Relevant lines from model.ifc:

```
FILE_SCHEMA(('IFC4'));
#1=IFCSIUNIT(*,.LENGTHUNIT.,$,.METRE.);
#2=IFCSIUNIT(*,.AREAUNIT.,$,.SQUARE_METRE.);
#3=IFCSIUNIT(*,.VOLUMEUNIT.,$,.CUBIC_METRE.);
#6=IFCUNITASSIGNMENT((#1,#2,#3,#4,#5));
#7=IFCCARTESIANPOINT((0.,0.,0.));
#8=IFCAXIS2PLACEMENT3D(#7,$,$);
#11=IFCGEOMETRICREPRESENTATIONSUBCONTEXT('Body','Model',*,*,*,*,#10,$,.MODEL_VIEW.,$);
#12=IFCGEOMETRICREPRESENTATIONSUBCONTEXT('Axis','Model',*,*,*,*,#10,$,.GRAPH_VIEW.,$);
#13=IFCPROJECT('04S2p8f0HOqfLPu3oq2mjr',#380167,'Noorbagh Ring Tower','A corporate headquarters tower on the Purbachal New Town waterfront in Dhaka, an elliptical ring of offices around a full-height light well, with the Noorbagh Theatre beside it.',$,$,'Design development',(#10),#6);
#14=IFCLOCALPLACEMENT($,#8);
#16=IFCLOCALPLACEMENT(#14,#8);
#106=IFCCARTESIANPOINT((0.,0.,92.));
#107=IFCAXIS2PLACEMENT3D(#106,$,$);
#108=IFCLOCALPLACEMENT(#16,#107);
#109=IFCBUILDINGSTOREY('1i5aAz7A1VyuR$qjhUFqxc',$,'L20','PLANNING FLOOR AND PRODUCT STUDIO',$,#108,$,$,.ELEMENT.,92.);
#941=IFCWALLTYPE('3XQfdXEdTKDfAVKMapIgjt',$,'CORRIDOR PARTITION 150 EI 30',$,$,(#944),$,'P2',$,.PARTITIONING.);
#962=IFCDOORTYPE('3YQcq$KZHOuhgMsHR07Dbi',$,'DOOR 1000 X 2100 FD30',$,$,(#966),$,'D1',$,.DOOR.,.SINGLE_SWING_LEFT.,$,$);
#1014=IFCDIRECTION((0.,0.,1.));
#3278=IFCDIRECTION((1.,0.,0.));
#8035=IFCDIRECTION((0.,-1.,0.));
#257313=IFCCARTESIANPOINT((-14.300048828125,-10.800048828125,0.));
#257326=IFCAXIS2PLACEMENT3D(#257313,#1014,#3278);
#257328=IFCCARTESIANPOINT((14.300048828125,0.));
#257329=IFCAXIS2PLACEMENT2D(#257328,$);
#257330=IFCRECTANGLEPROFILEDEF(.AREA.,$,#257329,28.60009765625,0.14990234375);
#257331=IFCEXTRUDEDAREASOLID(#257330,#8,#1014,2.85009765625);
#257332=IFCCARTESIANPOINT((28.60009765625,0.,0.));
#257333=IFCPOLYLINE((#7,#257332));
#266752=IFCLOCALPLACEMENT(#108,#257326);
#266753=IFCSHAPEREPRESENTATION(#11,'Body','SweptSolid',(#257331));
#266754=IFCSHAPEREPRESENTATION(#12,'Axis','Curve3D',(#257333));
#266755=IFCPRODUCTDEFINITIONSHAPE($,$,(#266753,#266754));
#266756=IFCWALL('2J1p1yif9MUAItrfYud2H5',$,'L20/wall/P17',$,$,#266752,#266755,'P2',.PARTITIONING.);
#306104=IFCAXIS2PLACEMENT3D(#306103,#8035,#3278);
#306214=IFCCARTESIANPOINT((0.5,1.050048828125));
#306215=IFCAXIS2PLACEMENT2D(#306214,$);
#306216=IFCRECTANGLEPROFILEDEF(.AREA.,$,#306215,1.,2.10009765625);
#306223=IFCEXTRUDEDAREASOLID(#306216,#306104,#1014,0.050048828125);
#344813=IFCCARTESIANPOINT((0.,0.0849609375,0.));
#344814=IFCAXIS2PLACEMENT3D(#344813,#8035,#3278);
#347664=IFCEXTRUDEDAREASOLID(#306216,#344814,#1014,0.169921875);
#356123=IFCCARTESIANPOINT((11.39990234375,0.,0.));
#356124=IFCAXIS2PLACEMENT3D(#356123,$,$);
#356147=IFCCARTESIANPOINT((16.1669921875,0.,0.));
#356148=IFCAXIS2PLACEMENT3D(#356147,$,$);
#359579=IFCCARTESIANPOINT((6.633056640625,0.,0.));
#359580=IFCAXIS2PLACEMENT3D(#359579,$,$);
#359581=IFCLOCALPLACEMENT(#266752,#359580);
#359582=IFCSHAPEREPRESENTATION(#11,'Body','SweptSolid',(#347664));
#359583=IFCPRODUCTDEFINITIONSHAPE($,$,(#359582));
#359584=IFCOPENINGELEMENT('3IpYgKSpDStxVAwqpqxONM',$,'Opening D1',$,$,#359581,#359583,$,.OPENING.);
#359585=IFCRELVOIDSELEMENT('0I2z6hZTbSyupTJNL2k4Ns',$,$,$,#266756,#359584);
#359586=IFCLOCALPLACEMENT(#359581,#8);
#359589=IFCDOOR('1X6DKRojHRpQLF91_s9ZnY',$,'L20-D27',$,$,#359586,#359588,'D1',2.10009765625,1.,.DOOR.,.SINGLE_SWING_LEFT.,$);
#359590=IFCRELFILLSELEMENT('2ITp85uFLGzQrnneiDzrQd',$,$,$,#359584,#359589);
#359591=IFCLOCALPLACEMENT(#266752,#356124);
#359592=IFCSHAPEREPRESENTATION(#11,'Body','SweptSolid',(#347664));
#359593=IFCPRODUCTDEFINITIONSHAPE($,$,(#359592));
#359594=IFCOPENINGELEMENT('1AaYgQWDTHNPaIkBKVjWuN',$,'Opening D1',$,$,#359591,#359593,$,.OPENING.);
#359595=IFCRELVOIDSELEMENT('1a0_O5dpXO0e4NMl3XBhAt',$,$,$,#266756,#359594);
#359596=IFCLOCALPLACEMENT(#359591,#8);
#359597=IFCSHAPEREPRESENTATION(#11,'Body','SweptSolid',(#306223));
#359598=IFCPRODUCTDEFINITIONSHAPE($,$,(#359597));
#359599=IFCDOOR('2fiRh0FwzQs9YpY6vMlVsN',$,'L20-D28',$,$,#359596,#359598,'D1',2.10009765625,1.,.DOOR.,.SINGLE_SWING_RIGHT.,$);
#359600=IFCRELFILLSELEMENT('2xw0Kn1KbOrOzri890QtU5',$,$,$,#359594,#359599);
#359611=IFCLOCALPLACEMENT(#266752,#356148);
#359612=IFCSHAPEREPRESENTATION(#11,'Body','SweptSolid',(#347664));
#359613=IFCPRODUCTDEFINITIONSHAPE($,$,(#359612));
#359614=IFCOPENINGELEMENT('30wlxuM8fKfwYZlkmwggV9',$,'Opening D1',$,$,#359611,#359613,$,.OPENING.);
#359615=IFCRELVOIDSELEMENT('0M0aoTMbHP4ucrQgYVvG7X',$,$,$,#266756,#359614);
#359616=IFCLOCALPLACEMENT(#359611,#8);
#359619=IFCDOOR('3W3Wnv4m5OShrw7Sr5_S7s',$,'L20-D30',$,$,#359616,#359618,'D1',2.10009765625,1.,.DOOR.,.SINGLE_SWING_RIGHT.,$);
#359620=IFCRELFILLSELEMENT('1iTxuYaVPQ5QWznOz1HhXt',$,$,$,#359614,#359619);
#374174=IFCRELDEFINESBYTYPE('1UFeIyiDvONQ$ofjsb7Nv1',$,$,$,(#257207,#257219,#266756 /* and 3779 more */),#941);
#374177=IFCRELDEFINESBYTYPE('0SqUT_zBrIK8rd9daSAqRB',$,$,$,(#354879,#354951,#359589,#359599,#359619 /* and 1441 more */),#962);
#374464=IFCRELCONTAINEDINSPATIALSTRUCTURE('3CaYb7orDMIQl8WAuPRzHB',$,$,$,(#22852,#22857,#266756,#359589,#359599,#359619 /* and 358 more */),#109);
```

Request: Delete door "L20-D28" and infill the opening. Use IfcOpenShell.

```python
import ifcopenshell
import ifcopenshell.api.feature
import ifcopenshell.api.root
import ifcopenshell.geom
import ifcopenshell.util.shape

model = ifcopenshell.open("model.ifc")
settings = ifcopenshell.geom.settings()


def volume(element):
    """Net volume in cubic metres, openings subtracted."""
    shape = ifcopenshell.geom.create_shape(settings, element)
    return ifcopenshell.util.shape.get_volume(shape.geometry)


door = model.by_guid("2fiRh0FwzQs9YpY6vMlVsN")
opening = door.FillsVoids[0].RelatingOpeningElement
wall = opening.VoidsElements[0].RelatingBuildingElement
before = volume(wall)

ifcopenshell.api.root.remove_product(model, product=door)
ifcopenshell.api.feature.remove_feature(model, feature=opening)

after = volume(wall)

print(f"wall volume {before:.3f} -> {after:.3f} m3")

model.write("model_rev.ifc")
```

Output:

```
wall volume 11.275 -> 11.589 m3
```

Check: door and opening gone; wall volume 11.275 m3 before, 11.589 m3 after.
